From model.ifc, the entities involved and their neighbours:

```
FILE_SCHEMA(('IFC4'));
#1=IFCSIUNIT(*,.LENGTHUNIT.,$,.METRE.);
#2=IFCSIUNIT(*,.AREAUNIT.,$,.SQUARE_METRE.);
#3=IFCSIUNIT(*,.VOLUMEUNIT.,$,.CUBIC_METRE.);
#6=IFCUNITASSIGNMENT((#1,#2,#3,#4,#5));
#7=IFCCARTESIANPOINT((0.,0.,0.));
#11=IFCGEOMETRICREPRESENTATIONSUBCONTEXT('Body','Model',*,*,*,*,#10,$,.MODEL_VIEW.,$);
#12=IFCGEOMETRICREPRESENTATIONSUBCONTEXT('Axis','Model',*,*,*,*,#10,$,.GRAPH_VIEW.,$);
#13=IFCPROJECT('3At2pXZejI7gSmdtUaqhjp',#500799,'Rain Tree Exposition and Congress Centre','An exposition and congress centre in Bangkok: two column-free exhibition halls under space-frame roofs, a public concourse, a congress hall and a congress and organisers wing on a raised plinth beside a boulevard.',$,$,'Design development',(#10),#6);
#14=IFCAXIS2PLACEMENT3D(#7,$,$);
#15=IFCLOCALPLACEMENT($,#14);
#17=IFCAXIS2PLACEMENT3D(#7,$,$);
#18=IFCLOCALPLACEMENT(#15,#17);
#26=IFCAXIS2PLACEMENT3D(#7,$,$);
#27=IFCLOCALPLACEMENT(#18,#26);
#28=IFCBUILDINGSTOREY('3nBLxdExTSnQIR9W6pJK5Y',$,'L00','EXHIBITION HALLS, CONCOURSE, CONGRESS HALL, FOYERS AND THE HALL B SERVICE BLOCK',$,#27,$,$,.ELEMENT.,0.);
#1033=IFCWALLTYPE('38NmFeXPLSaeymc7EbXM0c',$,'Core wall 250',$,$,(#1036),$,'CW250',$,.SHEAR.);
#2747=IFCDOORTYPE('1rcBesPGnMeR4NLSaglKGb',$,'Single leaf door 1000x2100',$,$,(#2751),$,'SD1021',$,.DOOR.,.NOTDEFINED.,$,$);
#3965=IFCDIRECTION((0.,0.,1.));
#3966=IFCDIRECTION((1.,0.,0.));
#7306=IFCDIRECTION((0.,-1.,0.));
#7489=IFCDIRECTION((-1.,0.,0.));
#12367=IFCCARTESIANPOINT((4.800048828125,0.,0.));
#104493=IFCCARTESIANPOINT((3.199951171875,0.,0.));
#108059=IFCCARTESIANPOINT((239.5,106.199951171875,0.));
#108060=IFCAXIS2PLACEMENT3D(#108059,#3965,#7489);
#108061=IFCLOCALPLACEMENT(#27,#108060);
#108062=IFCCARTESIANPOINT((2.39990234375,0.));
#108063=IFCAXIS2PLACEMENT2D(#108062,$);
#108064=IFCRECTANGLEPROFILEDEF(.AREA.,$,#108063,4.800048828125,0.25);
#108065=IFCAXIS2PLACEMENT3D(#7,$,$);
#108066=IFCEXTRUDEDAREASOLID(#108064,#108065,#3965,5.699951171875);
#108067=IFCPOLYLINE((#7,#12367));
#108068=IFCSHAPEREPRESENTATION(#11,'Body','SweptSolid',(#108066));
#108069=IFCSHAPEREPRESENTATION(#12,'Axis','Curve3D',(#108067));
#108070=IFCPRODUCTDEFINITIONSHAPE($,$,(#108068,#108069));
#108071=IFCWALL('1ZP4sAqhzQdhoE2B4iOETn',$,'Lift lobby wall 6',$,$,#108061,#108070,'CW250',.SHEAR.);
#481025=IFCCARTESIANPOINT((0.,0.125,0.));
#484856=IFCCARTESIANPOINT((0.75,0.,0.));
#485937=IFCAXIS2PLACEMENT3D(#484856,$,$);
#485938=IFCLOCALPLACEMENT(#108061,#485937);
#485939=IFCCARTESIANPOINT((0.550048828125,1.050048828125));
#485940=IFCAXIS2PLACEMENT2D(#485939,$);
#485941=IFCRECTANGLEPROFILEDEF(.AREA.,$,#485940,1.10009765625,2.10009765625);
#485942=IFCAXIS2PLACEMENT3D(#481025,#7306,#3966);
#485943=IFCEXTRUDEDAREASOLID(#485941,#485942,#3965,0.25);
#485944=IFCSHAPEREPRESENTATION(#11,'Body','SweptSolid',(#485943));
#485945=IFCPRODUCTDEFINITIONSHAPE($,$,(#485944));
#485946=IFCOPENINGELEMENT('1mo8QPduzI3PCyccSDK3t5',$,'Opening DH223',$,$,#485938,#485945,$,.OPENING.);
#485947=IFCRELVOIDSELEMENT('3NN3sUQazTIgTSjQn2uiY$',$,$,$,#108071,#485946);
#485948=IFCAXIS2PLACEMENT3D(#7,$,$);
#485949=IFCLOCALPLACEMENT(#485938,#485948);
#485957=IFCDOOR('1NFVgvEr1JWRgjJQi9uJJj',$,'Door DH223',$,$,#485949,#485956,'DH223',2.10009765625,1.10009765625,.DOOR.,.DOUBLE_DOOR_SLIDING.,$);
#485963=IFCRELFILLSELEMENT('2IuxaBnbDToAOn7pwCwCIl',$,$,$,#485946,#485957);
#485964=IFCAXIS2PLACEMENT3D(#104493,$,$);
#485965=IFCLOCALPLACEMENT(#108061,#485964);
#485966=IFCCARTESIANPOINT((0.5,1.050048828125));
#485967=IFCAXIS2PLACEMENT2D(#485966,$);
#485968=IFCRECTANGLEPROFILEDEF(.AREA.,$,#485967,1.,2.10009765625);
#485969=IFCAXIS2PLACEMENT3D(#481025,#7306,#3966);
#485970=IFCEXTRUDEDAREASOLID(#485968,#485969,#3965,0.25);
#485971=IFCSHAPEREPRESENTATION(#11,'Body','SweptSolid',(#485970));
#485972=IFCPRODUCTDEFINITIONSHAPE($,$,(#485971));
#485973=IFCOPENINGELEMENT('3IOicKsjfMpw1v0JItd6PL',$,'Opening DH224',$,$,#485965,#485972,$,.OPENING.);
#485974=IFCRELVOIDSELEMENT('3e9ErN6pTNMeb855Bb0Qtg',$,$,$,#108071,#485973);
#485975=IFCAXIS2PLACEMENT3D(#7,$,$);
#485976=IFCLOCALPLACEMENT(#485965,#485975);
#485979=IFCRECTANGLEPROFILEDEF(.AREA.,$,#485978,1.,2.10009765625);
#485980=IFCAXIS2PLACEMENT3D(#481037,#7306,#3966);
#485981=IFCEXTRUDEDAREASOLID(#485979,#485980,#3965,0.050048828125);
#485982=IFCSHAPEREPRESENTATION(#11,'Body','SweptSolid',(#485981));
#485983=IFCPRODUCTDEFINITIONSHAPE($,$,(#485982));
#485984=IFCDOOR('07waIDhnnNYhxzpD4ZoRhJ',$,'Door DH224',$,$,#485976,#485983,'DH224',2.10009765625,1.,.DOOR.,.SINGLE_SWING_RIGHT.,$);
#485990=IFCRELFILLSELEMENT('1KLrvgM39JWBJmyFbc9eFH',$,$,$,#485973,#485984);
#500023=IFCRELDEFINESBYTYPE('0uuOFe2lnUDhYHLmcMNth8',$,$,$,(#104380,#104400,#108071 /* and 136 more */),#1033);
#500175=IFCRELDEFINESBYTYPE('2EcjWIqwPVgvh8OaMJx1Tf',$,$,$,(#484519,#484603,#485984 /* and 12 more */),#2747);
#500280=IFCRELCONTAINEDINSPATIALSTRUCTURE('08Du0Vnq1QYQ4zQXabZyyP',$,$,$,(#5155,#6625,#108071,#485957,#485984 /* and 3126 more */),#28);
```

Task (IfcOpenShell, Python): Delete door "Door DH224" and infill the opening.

```python
import ifcopenshell
import ifcopenshell.api.feature
import ifcopenshell.api.root
import ifcopenshell.geom
import ifcopenshell.util.shape

model = ifcopenshell.open("model.ifc")
settings = ifcopenshell.geom.settings()


def volume(element):
    """Net volume in cubic metres, openings subtracted."""
    shape = ifcopenshell.geom.create_shape(settings, element)
    return ifcopenshell.util.shape.get_volume(shape.geometry)


door = model.by_guid("07waIDhnnNYhxzpD4ZoRhJ")
opening = door.FillsVoids[0].RelatingOpeningElement
wall = opening.VoidsElements[0].RelatingBuildingElement
before = volume(wall)

ifcopenshell.api.root.remove_product(model, product=door)
ifcopenshell.api.feature.remove_feature(model, feature=opening)

after = volume(wall)

print(f"wall volume {before:.3f} -> {after:.3f} m3")

model.write("model_updated.ifc")
```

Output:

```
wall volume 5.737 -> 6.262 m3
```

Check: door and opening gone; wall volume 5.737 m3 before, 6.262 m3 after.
